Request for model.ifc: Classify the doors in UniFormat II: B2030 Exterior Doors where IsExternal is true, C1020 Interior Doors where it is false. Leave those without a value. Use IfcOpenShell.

First a look at what the model holds.

```python
import ifcopenshell
import ifcopenshell.util.element

model = ifcopenshell.open("model.ifc")
print(model.schema)
print("classifications:", [c.Name for c in model.by_type("IfcClassification")])
values = [ifcopenshell.util.element.get_pset(e, "Pset_DoorCommon", "IsExternal") for e in model.by_type("IfcDoor")]
for value in (True, False, None):
    print("IsExternal", value, values.count(value))
```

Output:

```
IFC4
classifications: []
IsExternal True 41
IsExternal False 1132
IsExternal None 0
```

```python
import ifcopenshell
import ifcopenshell.api.classification
import ifcopenshell.util.element

model = ifcopenshell.open("model.ifc")

system = ifcopenshell.api.classification.add_classification(model, classification="UniFormat II")

doors = model.by_type("IfcDoor")
external = {e: ifcopenshell.util.element.get_pset(e, "Pset_DoorCommon", "IsExternal") for e in doors}
for flag, code, name in ((True, "B2030", "Exterior Doors"), (False, "C1020", "Interior Doors")):
    products = [e for e in doors if external[e] is flag]
    ifcopenshell.api.classification.add_reference(
        model, products=products, classification=system, identification=code, name=name
    )
    print(code, len(products))

model.write("model_updated.ifc")
```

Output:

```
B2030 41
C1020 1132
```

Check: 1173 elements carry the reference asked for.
